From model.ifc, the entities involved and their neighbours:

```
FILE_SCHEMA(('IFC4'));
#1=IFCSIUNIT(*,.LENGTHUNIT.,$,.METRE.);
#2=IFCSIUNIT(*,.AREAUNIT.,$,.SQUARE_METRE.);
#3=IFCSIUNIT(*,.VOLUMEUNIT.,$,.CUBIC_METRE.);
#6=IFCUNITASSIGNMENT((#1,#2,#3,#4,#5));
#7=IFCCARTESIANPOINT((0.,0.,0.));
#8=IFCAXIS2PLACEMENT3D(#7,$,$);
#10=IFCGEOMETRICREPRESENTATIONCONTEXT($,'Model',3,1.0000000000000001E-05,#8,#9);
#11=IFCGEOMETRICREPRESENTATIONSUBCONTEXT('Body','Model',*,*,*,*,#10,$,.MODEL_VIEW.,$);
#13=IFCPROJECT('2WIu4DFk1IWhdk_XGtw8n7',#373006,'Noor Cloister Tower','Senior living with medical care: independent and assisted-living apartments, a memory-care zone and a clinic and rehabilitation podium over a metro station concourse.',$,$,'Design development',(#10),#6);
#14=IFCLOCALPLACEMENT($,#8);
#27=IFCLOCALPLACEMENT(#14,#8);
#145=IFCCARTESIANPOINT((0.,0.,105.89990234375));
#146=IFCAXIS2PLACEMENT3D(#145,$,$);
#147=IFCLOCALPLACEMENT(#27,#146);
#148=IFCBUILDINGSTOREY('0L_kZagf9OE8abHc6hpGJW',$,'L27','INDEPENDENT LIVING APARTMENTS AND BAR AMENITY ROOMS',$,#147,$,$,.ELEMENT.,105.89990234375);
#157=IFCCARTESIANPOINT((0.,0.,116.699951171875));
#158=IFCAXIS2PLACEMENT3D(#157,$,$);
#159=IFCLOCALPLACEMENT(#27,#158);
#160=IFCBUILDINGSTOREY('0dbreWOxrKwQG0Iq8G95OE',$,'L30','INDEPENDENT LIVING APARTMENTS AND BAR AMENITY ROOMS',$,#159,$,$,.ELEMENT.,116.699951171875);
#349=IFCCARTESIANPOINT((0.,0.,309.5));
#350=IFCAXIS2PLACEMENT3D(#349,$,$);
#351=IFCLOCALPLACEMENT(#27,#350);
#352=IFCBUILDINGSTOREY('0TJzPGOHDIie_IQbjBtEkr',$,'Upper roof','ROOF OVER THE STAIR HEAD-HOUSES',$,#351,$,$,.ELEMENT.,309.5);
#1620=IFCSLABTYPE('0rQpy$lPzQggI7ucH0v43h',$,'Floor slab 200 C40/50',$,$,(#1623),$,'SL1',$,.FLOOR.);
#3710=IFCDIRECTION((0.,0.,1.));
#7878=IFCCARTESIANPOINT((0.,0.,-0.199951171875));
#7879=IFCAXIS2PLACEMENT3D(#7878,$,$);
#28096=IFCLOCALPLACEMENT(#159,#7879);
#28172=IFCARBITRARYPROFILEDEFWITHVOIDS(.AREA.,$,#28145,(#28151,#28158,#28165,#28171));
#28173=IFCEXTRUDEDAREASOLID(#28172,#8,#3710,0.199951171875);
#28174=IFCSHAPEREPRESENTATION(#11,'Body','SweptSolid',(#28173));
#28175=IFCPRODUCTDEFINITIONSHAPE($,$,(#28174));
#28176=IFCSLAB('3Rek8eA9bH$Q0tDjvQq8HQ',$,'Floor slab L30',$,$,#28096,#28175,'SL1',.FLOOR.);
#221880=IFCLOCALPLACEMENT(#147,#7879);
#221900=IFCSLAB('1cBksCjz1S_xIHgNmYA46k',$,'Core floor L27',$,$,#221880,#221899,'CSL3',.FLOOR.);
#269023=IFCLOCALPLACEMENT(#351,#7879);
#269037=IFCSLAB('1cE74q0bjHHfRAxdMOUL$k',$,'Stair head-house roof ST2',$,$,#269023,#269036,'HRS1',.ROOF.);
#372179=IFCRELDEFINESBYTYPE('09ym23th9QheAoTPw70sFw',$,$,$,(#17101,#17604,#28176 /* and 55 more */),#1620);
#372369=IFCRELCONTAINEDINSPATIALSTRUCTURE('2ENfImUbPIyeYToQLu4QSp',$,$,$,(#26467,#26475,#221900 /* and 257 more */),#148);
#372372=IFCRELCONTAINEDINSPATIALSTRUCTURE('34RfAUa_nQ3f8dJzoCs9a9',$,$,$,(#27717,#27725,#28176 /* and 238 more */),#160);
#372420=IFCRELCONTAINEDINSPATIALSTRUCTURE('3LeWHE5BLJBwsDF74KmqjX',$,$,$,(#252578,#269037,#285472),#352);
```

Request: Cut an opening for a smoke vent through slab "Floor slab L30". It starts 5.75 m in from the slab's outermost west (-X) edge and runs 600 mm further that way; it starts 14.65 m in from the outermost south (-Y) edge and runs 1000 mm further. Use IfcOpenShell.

```python
import numpy as np
import ifcopenshell
import ifcopenshell.api.feature
import ifcopenshell.api.geometry
import ifcopenshell.api.root
import ifcopenshell.geom
import ifcopenshell.util.placement
import ifcopenshell.util.representation
import ifcopenshell.util.shape
import ifcopenshell.util.unit

model = ifcopenshell.open("model.ifc")
unit_scale = ifcopenshell.util.unit.calculate_unit_scale(model)
settings = ifcopenshell.geom.settings()


def volume(element):
    """Net volume in cubic metres, openings subtracted."""
    shape = ifcopenshell.geom.create_shape(settings, element)
    return ifcopenshell.util.shape.get_volume(shape.geometry)


slab = model.by_guid("3Rek8eA9bH$Q0tDjvQq8HQ")
before = volume(slab)

# Extent in the slab's own axes, in metres. The edges named are its -X and -Y sides.
slab_shape = ifcopenshell.geom.create_shape(settings, slab)
vertices = ifcopenshell.util.shape.get_vertices(slab_shape.geometry)
x_min, y_min, bottom = vertices.min(axis=0)
top = vertices[:, 2].max()

opening = ifcopenshell.api.root.create_entity(model, ifc_class="IfcOpeningElement", name="Smoke vent opening", predefined_type="OPENING")
context = ifcopenshell.util.representation.get_context(model, "Model", "Body", "MODEL_VIEW")
width, depth = 0.6, 1
outline = [(0.0, 0.0), (width, 0.0), (width, depth), (0.0, depth), (0.0, 0.0)]
# Overshoot both faces by 50 mm so the cut is clean.
shape = ifcopenshell.api.geometry.add_slab_representation(
    model, context=context, depth=top - bottom + 0.1, polyline=outline
)
ifcopenshell.api.geometry.assign_representation(model, product=opening, representation=shape)

matrix = ifcopenshell.util.placement.get_local_placement(slab.ObjectPlacement)
matrix[:, 3] = matrix @ np.append(np.array([x_min + 5.75, y_min + 14.65, bottom - 0.05]) / unit_scale, 1.0)
ifcopenshell.api.geometry.edit_object_placement(model, product=opening, matrix=matrix, is_si=False)
ifcopenshell.api.feature.add_feature(model, feature=opening, element=slab)

after = volume(slab)

print(f"slab volume {before:.3f} -> {after:.3f} m3")

model.write("model-out.ifc")
```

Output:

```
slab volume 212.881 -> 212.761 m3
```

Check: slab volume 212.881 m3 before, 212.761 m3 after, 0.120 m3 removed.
